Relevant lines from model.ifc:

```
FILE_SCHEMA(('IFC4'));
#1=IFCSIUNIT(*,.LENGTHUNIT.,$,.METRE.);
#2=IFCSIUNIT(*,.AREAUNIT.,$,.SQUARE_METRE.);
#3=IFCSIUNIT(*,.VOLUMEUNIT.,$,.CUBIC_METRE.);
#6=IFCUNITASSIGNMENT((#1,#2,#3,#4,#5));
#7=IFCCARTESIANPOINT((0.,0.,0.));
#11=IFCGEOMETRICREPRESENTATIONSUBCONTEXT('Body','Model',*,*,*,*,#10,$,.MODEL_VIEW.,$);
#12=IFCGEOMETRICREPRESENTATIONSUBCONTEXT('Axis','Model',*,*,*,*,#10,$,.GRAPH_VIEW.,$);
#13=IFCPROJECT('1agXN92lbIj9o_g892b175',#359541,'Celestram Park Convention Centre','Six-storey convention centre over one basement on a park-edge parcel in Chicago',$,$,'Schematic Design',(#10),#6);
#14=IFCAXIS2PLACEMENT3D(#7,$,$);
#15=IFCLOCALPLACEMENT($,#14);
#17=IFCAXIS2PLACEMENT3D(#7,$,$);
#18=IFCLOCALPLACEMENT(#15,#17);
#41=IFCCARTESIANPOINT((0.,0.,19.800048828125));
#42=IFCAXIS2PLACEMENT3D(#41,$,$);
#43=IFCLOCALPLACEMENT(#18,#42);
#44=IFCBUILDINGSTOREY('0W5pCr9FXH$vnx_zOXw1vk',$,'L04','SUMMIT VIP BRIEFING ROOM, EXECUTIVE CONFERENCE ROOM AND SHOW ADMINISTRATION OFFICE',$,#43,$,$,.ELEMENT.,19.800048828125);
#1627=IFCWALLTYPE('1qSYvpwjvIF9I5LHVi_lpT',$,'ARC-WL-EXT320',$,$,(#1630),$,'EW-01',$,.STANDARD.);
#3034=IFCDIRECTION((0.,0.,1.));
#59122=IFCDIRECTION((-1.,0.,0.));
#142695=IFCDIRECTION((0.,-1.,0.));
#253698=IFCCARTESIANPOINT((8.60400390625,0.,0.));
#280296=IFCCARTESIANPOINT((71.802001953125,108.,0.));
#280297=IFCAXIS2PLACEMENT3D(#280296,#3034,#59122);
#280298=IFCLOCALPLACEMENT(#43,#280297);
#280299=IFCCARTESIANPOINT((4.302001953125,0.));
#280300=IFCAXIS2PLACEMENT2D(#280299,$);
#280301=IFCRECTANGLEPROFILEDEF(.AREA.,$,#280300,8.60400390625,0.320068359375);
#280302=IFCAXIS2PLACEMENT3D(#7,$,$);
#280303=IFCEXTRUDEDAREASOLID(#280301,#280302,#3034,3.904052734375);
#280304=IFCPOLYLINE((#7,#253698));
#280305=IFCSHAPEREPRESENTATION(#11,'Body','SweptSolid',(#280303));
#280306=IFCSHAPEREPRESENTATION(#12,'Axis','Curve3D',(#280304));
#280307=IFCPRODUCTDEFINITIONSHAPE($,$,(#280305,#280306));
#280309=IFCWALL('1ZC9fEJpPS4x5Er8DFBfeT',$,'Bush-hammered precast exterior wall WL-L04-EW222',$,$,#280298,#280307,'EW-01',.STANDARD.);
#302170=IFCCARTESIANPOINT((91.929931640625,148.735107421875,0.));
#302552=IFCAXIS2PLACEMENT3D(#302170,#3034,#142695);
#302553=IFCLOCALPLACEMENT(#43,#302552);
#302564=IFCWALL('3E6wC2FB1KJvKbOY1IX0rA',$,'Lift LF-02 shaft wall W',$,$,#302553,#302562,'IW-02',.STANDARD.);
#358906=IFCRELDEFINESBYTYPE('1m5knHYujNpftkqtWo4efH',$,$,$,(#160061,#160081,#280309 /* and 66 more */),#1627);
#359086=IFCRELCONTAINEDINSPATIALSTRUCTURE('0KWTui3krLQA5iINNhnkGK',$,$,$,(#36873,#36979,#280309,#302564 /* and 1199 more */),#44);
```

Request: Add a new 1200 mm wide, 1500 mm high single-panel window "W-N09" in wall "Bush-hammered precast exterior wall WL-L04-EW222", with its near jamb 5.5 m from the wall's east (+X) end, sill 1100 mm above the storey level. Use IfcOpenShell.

```python
import numpy as np
import ifcopenshell
import ifcopenshell.api.feature
import ifcopenshell.api.geometry
import ifcopenshell.api.root
import ifcopenshell.api.spatial
import ifcopenshell.geom
import ifcopenshell.util.element
import ifcopenshell.util.placement
import ifcopenshell.util.representation
import ifcopenshell.util.shape
import ifcopenshell.util.unit

model = ifcopenshell.open("model.ifc")
unit_scale = ifcopenshell.util.unit.calculate_unit_scale(model)
settings = ifcopenshell.geom.settings()


def volume(element):
    """Net volume in cubic metres, openings subtracted."""
    shape = ifcopenshell.geom.create_shape(settings, element)
    return ifcopenshell.util.shape.get_volume(shape.geometry)


wall = model.by_id(280309)
storey = ifcopenshell.util.element.get_container(wall, ifc_class="IfcBuildingStorey")
context = ifcopenshell.util.representation.get_context(model, "Model", "Body", "MODEL_VIEW")
before = volume(wall)

width, height, from_end, sill = 1.2, 1.5, 5.5, 1.1  # metres

# The wall runs along its own X axis, and the end named is its -X end.
wall_shape = ifcopenshell.geom.create_shape(settings, wall)
x, y, z = ifcopenshell.util.shape.get_vertices(wall_shape.geometry).T
start = x.min() + from_end
face, thickness = float(y.min()), float(y.max() - y.min())
wall_matrix = ifcopenshell.util.placement.get_local_placement(wall.ObjectPlacement)
level = ifcopenshell.util.placement.get_local_placement(storey.ObjectPlacement)[2, 3]


def in_wall(x, y):
    """Placement at x, y metres in the wall's axes, at sill height."""
    matrix = wall_matrix.copy()
    matrix[:, 3] = wall_matrix @ np.array([x / unit_scale, y / unit_scale, 0.0, 1.0])
    matrix[2, 3] = level + sill / unit_scale
    return matrix


# Opening: a box that overshoots both wall faces by 50 mm.
opening = ifcopenshell.api.root.create_entity(model, ifc_class="IfcOpeningElement", predefined_type="OPENING")
box = ifcopenshell.api.geometry.add_wall_representation(
    model, context=context, length=width, height=height, thickness=thickness + 0.1
)
ifcopenshell.api.geometry.assign_representation(model, product=opening, representation=box)
ifcopenshell.api.geometry.edit_object_placement(model, product=opening, matrix=in_wall(start, face - 0.05), is_si=False)
ifcopenshell.api.feature.add_feature(model, feature=opening, element=wall)

window = ifcopenshell.api.root.create_entity(model, ifc_class="IfcWindow", name="W-N09", predefined_type="WINDOW")
window.OverallWidth, window.OverallHeight = width / unit_scale, height / unit_scale
window.PartitioningType = "SINGLE_PANEL"
body = ifcopenshell.api.geometry.add_window_representation(
    model,
    context=context,
    overall_width=window.OverallWidth,
    overall_height=window.OverallHeight,
    partition_type="SINGLE_PANEL",
)
ifcopenshell.api.geometry.assign_representation(model, product=window, representation=body)
ifcopenshell.api.spatial.assign_container(model, products=[window], relating_structure=storey)
ifcopenshell.api.feature.add_filling(model, opening=opening, element=window)

# Centre the window in the wall's thickness.
ifcopenshell.api.geometry.edit_object_placement(model, product=window, matrix=in_wall(start, face), is_si=False)
window_shape = ifcopenshell.geom.create_shape(settings, window)
depth = ifcopenshell.util.shape.get_vertices(window_shape.geometry)[:, 1]
offset = face + thickness / 2 - (depth.min() + depth.max()) / 2
ifcopenshell.api.geometry.edit_object_placement(model, product=window, matrix=in_wall(start, offset), is_si=False)

after = volume(wall)

print(f"wall volume {before:.3f} -> {after:.3f} m3")

model.write("model_updated.ifc")
```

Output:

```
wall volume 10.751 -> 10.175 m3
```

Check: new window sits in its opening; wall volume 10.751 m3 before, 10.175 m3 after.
